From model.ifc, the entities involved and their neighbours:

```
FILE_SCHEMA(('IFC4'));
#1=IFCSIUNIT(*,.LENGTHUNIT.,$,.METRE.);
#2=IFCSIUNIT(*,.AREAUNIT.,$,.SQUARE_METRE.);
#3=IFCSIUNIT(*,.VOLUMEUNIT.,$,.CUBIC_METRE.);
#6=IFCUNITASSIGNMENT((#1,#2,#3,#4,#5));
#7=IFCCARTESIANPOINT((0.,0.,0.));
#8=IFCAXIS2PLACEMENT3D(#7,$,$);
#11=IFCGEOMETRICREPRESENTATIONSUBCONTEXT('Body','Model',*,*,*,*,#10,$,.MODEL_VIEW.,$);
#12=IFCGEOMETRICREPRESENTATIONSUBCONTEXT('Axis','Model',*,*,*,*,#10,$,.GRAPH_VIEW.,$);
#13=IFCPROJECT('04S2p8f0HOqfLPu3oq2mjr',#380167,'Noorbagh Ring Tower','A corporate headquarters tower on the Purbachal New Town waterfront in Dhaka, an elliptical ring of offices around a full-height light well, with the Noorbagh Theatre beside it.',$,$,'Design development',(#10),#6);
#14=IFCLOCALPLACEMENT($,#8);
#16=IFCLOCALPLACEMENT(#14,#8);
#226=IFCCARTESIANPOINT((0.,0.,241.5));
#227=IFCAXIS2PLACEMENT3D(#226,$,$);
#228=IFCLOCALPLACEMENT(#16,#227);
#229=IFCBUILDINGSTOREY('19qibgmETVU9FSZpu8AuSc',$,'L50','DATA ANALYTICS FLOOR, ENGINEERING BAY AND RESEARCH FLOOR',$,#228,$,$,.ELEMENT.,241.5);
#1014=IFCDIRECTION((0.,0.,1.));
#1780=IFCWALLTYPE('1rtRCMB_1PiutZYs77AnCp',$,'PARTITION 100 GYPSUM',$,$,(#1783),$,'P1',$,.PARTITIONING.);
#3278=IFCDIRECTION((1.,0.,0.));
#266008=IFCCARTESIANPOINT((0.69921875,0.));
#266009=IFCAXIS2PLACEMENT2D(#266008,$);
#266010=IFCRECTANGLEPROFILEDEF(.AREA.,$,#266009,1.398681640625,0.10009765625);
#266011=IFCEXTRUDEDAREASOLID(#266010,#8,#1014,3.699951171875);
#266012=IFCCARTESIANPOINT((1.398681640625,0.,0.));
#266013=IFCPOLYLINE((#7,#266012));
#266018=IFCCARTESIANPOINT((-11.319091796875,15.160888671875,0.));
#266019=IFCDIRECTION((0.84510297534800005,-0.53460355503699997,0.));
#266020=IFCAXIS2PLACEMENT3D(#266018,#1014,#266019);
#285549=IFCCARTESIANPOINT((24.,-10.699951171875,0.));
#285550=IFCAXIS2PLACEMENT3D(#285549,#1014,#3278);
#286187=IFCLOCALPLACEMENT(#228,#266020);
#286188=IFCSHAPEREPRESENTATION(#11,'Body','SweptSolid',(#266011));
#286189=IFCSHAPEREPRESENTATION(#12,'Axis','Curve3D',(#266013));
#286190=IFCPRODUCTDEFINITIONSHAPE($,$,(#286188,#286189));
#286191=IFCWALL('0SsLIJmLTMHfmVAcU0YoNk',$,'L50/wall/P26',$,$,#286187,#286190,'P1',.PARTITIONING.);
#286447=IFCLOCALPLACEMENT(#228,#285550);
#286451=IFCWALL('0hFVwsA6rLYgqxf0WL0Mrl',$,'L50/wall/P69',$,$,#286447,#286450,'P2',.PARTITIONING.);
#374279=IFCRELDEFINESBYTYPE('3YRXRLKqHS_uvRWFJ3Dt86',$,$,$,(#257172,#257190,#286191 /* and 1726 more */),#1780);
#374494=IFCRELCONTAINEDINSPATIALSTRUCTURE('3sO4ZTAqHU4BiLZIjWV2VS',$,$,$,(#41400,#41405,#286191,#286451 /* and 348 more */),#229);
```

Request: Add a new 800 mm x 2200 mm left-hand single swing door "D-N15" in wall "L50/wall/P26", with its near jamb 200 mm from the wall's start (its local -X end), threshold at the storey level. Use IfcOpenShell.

```python
import numpy as np
import ifcopenshell
import ifcopenshell.api.feature
import ifcopenshell.api.geometry
import ifcopenshell.api.root
import ifcopenshell.api.spatial
import ifcopenshell.geom
import ifcopenshell.util.element
import ifcopenshell.util.placement
import ifcopenshell.util.representation
import ifcopenshell.util.shape
import ifcopenshell.util.unit

model = ifcopenshell.open("model.ifc")
unit_scale = ifcopenshell.util.unit.calculate_unit_scale(model)
settings = ifcopenshell.geom.settings()


def volume(element):
    """Net volume in cubic metres, openings subtracted."""
    shape = ifcopenshell.geom.create_shape(settings, element)
    return ifcopenshell.util.shape.get_volume(shape.geometry)


wall = model.by_guid("0SsLIJmLTMHfmVAcU0YoNk")
storey = ifcopenshell.util.element.get_container(wall, ifc_class="IfcBuildingStorey")
context = ifcopenshell.util.representation.get_context(model, "Model", "Body", "MODEL_VIEW")
before = volume(wall)

width, height, from_end, sill = 0.8, 2.2, 0.2, 0.0  # metres

# The wall runs along its own X axis, and the end named is its -X end.
wall_shape = ifcopenshell.geom.create_shape(settings, wall)
x, y, z = ifcopenshell.util.shape.get_vertices(wall_shape.geometry).T
start = x.min() + from_end
face, thickness = float(y.min()), float(y.max() - y.min())
wall_matrix = ifcopenshell.util.placement.get_local_placement(wall.ObjectPlacement)
level = ifcopenshell.util.placement.get_local_placement(storey.ObjectPlacement)[2, 3]


def in_wall(x, y):
    """Placement at x, y metres in the wall's axes, at sill height."""
    matrix = wall_matrix.copy()
    matrix[:, 3] = wall_matrix @ np.array([x / unit_scale, y / unit_scale, 0.0, 1.0])
    matrix[2, 3] = level + sill / unit_scale
    return matrix


# Opening: a box that overshoots both wall faces by 50 mm.
opening = ifcopenshell.api.root.create_entity(model, ifc_class="IfcOpeningElement", predefined_type="OPENING")
box = ifcopenshell.api.geometry.add_wall_representation(
    model, context=context, length=width, height=height, thickness=thickness + 0.1
)
ifcopenshell.api.geometry.assign_representation(model, product=opening, representation=box)
ifcopenshell.api.geometry.edit_object_placement(model, product=opening, matrix=in_wall(start, face - 0.05), is_si=False)
ifcopenshell.api.feature.add_feature(model, feature=opening, element=wall)

door = ifcopenshell.api.root.create_entity(model, ifc_class="IfcDoor", name="D-N15", predefined_type="DOOR")
door.OverallWidth, door.OverallHeight = width / unit_scale, height / unit_scale
door.OperationType = "SINGLE_SWING_LEFT"
body = ifcopenshell.api.geometry.add_door_representation(
    model,
    context=context,
    overall_width=door.OverallWidth,
    overall_height=door.OverallHeight,
    operation_type="SINGLE_SWING_LEFT",
    lining_properties={"LiningDepth": thickness / unit_scale, "ThresholdDepth": thickness / unit_scale},
)
ifcopenshell.api.geometry.assign_representation(model, product=door, representation=body)
ifcopenshell.api.spatial.assign_container(model, products=[door], relating_structure=storey)
ifcopenshell.api.feature.add_filling(model, opening=opening, element=door)

# The lining spans the wall, so the door starts at the wall face.
ifcopenshell.api.geometry.edit_object_placement(model, product=door, matrix=in_wall(start, face), is_si=False)

after = volume(wall)

print(f"wall volume {before:.3f} -> {after:.3f} m3")

model.write("model_updated.ifc")
```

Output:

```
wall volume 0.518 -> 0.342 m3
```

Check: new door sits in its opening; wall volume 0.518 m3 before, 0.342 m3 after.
